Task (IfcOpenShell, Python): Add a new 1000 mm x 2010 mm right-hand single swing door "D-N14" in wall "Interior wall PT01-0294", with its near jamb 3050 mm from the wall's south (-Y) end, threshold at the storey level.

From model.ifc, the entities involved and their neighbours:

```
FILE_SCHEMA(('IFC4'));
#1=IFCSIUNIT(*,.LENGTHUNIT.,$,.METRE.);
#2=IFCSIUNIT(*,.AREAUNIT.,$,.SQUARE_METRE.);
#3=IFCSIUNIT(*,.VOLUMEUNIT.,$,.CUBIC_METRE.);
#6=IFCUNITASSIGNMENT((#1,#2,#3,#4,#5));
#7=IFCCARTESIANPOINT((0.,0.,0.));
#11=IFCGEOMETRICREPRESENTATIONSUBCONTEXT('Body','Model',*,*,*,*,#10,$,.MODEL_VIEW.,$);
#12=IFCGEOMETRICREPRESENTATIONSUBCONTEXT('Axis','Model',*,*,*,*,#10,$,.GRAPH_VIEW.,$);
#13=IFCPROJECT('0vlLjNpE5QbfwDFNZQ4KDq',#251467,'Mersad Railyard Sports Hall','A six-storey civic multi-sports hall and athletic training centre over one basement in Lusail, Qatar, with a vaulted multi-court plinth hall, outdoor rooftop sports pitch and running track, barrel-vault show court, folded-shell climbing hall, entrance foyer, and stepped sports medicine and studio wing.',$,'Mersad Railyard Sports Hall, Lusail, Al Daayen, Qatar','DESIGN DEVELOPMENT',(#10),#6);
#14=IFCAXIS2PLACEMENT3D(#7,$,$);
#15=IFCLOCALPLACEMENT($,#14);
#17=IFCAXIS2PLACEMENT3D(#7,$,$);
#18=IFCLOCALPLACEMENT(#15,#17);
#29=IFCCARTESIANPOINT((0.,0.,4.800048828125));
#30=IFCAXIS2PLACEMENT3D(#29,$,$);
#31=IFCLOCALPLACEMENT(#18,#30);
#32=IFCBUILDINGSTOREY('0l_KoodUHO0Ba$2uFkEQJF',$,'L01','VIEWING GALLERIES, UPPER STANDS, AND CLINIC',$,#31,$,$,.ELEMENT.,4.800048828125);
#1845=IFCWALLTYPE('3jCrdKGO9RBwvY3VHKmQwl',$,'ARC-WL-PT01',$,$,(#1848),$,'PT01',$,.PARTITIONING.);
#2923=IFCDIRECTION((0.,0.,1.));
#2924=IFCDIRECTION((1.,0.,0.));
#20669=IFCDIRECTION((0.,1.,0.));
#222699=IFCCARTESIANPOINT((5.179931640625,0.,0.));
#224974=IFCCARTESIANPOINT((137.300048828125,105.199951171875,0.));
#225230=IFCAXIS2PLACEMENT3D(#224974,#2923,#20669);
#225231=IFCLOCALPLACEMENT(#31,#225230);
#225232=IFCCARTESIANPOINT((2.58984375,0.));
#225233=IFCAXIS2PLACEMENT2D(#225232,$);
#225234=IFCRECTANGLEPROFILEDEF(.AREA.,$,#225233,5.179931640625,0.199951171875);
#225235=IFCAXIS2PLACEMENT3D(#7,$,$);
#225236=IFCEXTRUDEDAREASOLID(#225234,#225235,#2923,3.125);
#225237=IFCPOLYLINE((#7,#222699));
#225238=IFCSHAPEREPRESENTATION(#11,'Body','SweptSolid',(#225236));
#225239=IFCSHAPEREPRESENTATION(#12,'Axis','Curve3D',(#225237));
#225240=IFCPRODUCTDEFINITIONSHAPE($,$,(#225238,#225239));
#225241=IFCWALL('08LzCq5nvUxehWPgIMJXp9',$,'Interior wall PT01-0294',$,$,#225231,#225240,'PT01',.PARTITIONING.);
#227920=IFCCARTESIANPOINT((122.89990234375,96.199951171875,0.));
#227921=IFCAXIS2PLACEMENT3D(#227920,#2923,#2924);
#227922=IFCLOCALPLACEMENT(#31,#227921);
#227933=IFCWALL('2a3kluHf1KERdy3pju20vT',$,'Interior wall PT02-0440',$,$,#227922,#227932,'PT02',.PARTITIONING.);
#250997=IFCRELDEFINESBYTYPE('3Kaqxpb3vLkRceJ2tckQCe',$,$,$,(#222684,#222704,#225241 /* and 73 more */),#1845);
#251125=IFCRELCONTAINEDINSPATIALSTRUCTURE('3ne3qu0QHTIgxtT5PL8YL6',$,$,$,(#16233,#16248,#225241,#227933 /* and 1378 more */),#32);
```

```python
import numpy as np
import ifcopenshell
import ifcopenshell.api.feature
import ifcopenshell.api.geometry
import ifcopenshell.api.root
import ifcopenshell.api.spatial
import ifcopenshell.geom
import ifcopenshell.util.element
import ifcopenshell.util.placement
import ifcopenshell.util.representation
import ifcopenshell.util.shape
import ifcopenshell.util.unit

model = ifcopenshell.open("model.ifc")
unit_scale = ifcopenshell.util.unit.calculate_unit_scale(model)
settings = ifcopenshell.geom.settings()


def volume(element):
    """Net volume in cubic metres, openings subtracted."""
    shape = ifcopenshell.geom.create_shape(settings, element)
    return ifcopenshell.util.shape.get_volume(shape.geometry)


wall = model.by_id(225241)
storey = ifcopenshell.util.element.get_container(wall, ifc_class="IfcBuildingStorey")
context = ifcopenshell.util.representation.get_context(model, "Model", "Body", "MODEL_VIEW")
before = volume(wall)

width, height, from_end, sill = 1, 2.01, 3.05, 0.0  # metres

# The wall runs along its own X axis, and the end named is its -X end.
wall_shape = ifcopenshell.geom.create_shape(settings, wall)
x, y, z = ifcopenshell.util.shape.get_vertices(wall_shape.geometry).T
start = x.min() + from_end
face, thickness = float(y.min()), float(y.max() - y.min())
wall_matrix = ifcopenshell.util.placement.get_local_placement(wall.ObjectPlacement)
level = ifcopenshell.util.placement.get_local_placement(storey.ObjectPlacement)[2, 3]


def in_wall(x, y):
    """Placement at x, y metres in the wall's axes, at sill height."""
    matrix = wall_matrix.copy()
    matrix[:, 3] = wall_matrix @ np.array([x / unit_scale, y / unit_scale, 0.0, 1.0])
    matrix[2, 3] = level + sill / unit_scale
    return matrix


# Opening: a box that overshoots both wall faces by 50 mm.
opening = ifcopenshell.api.root.create_entity(model, ifc_class="IfcOpeningElement", predefined_type="OPENING")
box = ifcopenshell.api.geometry.add_wall_representation(
    model, context=context, length=width, height=height, thickness=thickness + 0.1
)
ifcopenshell.api.geometry.assign_representation(model, product=opening, representation=box)
ifcopenshell.api.geometry.edit_object_placement(model, product=opening, matrix=in_wall(start, face - 0.05), is_si=False)
ifcopenshell.api.feature.add_feature(model, feature=opening, element=wall)

door = ifcopenshell.api.root.create_entity(model, ifc_class="IfcDoor", name="D-N14", predefined_type="DOOR")
door.OverallWidth, door.OverallHeight = width / unit_scale, height / unit_scale
door.OperationType = "SINGLE_SWING_RIGHT"
body = ifcopenshell.api.geometry.add_door_representation(
    model,
    context=context,
    overall_width=door.OverallWidth,
    overall_height=door.OverallHeight,
    operation_type="SINGLE_SWING_RIGHT",
    lining_properties={"LiningDepth": thickness / unit_scale, "ThresholdDepth": thickness / unit_scale},
)
ifcopenshell.api.geometry.assign_representation(model, product=door, representation=body)
ifcopenshell.api.spatial.assign_container(model, products=[door], relating_structure=storey)
ifcopenshell.api.feature.add_filling(model, opening=opening, element=door)

# The lining spans the wall, so the door starts at the wall face.
ifcopenshell.api.geometry.edit_object_placement(model, product=door, matrix=in_wall(start, face), is_si=False)

after = volume(wall)

print(f"wall volume {before:.3f} -> {after:.3f} m3")

model.write("model-out.ifc")
```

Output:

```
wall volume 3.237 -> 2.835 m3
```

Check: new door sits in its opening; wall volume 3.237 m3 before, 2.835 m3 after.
